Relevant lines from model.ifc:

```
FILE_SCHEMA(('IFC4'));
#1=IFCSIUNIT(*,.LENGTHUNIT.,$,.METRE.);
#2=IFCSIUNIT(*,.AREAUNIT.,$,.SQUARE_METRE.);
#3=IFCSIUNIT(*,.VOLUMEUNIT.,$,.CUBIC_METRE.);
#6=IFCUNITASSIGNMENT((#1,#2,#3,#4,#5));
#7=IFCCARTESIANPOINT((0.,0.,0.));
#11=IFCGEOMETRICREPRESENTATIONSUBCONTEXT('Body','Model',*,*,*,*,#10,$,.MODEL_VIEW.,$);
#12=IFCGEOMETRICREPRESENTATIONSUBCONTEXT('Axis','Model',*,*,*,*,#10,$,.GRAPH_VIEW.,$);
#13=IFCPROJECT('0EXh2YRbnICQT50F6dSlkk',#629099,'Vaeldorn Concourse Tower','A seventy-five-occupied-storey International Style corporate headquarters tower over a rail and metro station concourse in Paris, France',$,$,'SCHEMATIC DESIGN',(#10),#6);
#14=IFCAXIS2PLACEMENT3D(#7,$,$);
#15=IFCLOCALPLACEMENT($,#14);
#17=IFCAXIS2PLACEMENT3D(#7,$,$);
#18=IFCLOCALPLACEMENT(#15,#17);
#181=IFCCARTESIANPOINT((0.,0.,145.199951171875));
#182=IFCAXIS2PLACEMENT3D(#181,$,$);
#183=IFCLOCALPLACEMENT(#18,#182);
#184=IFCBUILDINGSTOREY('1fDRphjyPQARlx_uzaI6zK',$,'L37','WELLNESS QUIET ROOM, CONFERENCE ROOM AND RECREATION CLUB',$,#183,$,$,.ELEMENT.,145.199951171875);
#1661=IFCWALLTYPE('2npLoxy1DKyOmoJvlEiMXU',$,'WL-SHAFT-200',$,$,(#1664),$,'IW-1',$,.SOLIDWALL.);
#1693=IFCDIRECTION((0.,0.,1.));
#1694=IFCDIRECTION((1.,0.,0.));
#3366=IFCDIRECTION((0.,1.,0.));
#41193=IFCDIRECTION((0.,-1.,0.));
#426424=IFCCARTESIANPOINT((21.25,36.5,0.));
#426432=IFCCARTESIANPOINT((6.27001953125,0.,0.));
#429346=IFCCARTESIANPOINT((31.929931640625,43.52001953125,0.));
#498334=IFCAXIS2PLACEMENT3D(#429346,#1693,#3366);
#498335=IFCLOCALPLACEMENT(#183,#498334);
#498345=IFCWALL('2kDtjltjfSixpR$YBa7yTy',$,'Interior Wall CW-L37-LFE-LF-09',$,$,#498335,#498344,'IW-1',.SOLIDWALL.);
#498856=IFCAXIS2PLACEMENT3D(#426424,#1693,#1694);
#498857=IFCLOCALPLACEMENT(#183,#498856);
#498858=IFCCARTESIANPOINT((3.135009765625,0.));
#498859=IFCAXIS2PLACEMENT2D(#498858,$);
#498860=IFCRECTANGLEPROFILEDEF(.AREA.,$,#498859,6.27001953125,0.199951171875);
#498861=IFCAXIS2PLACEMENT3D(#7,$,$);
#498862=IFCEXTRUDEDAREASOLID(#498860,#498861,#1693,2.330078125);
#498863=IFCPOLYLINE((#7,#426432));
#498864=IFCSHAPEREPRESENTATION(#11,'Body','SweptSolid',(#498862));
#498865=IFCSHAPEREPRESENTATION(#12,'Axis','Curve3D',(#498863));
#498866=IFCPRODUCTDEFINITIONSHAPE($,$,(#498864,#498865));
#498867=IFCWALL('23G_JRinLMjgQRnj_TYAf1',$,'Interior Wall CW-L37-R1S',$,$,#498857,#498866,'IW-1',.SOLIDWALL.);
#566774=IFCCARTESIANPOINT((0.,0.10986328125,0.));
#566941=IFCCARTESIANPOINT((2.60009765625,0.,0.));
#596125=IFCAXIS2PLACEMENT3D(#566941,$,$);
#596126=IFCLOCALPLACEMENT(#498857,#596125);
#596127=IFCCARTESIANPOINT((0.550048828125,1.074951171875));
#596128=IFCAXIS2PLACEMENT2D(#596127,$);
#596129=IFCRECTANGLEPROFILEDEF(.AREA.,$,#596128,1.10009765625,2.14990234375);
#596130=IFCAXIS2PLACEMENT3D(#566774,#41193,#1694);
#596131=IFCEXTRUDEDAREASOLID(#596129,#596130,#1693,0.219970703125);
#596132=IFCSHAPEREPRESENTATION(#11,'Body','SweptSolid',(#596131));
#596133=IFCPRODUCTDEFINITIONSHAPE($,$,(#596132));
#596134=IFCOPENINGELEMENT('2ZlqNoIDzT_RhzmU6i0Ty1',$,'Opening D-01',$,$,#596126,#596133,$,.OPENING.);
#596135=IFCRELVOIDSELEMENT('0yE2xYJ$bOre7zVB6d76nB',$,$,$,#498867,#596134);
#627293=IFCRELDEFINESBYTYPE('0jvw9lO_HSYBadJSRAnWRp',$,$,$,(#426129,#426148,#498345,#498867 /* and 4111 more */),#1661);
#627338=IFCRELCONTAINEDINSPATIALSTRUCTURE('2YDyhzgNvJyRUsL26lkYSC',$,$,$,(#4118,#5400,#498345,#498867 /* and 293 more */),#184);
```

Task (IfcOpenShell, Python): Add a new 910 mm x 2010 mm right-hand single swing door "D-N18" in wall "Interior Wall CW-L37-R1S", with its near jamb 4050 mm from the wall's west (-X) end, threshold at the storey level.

```python
import numpy as np
import ifcopenshell
import ifcopenshell.api.feature
import ifcopenshell.api.geometry
import ifcopenshell.api.root
import ifcopenshell.api.spatial
import ifcopenshell.geom
import ifcopenshell.util.element
import ifcopenshell.util.placement
import ifcopenshell.util.representation
import ifcopenshell.util.shape
import ifcopenshell.util.unit

model = ifcopenshell.open("model.ifc")
unit_scale = ifcopenshell.util.unit.calculate_unit_scale(model)
settings = ifcopenshell.geom.settings()


def volume(element):
    """Net volume in cubic metres, openings subtracted."""
    shape = ifcopenshell.geom.create_shape(settings, element)
    return ifcopenshell.util.shape.get_volume(shape.geometry)


wall = model.by_id(498867)
storey = ifcopenshell.util.element.get_container(wall, ifc_class="IfcBuildingStorey")
context = ifcopenshell.util.representation.get_context(model, "Model", "Body", "MODEL_VIEW")
before = volume(wall)

width, height, from_end, sill = 0.91, 2.01, 4.05, 0.0  # metres

# The wall runs along its own X axis, and the end named is its -X end.
wall_shape = ifcopenshell.geom.create_shape(settings, wall)
x, y, z = ifcopenshell.util.shape.get_vertices(wall_shape.geometry).T
start = x.min() + from_end
face, thickness = float(y.min()), float(y.max() - y.min())
wall_matrix = ifcopenshell.util.placement.get_local_placement(wall.ObjectPlacement)
level = ifcopenshell.util.placement.get_local_placement(storey.ObjectPlacement)[2, 3]


def in_wall(x, y):
    """Placement at x, y metres in the wall's axes, at sill height."""
    matrix = wall_matrix.copy()
    matrix[:, 3] = wall_matrix @ np.array([x / unit_scale, y / unit_scale, 0.0, 1.0])
    matrix[2, 3] = level + sill / unit_scale
    return matrix


# Opening: a box that overshoots both wall faces by 50 mm.
opening = ifcopenshell.api.root.create_entity(model, ifc_class="IfcOpeningElement", predefined_type="OPENING")
box = ifcopenshell.api.geometry.add_wall_representation(
    model, context=context, length=width, height=height, thickness=thickness + 0.1
)
ifcopenshell.api.geometry.assign_representation(model, product=opening, representation=box)
ifcopenshell.api.geometry.edit_object_placement(model, product=opening, matrix=in_wall(start, face - 0.05), is_si=False)
ifcopenshell.api.feature.add_feature(model, feature=opening, element=wall)

door = ifcopenshell.api.root.create_entity(model, ifc_class="IfcDoor", name="D-N18", predefined_type="DOOR")
door.OverallWidth, door.OverallHeight = width / unit_scale, height / unit_scale
door.OperationType = "SINGLE_SWING_RIGHT"
body = ifcopenshell.api.geometry.add_door_representation(
    model,
    context=context,
    overall_width=door.OverallWidth,
    overall_height=door.OverallHeight,
    operation_type="SINGLE_SWING_RIGHT",
    lining_properties={"LiningDepth": thickness / unit_scale, "ThresholdDepth": thickness / unit_scale},
)
ifcopenshell.api.geometry.assign_representation(model, product=door, representation=body)
ifcopenshell.api.spatial.assign_container(model, products=[door], relating_structure=storey)
ifcopenshell.api.feature.add_filling(model, opening=opening, element=door)

# The lining spans the wall, so the door starts at the wall face.
ifcopenshell.api.geometry.edit_object_placement(model, product=door, matrix=in_wall(start, face), is_si=False)

after = volume(wall)

print(f"wall volume {before:.3f} -> {after:.3f} m3")

model.write("model_v2.ifc")
```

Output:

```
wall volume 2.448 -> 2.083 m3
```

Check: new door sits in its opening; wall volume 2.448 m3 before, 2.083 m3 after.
